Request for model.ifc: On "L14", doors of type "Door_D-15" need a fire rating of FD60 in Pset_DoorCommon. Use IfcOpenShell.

First a look at what the model holds.

```python
import ifcopenshell
import ifcopenshell.util.element

model = ifcopenshell.open("model.ifc")
print(model.schema)
storey = next(s for s in model.by_type("IfcBuildingStorey") if s.Name == "L14")
doors = [e for e in ifcopenshell.util.element.get_decomposition(storey) if e.is_a("IfcDoor")]
seen = {}
for e in doors:
    element_type = ifcopenshell.util.element.get_type(e)
    key = (element_type.Name if element_type != e and element_type else None, ifcopenshell.util.element.get_pset(e, "Pset_DoorCommon", "FireRating"))
    seen[key] = seen.get(key, 0) + 1
for (name, value), count in sorted(seen.items(), key=str):
    print(count, "x", name, "|", value)
```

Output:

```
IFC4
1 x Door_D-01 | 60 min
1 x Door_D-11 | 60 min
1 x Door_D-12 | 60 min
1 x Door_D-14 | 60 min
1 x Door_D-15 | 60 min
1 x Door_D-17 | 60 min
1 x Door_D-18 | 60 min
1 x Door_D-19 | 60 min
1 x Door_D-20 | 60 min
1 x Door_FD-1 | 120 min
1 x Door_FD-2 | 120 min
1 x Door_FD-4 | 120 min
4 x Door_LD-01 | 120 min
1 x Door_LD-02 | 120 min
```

```python
import ifcopenshell
import ifcopenshell.api.pset
import ifcopenshell.util.element

model = ifcopenshell.open("model.ifc")

storey = next(s for s in model.by_type("IfcBuildingStorey") if s.Name == "L14")
doors = [e for e in ifcopenshell.util.element.get_decomposition(storey) if e.is_a("IfcDoor")]

count = 0
for e in doors:
    element_type = ifcopenshell.util.element.get_type(e)
    if element_type in (None, e) or element_type.Name != "Door_D-15":
        continue
    # add_pset returns the element's existing set when there is one.
    pset = ifcopenshell.api.pset.add_pset(model, product=e, name="Pset_DoorCommon")
    ifcopenshell.api.pset.edit_pset(model, pset=pset, properties={"FireRating": "FD60"})
    count += 1

print(count, "doors updated")

model.write("model_edited.ifc")
```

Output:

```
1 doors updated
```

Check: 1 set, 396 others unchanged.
